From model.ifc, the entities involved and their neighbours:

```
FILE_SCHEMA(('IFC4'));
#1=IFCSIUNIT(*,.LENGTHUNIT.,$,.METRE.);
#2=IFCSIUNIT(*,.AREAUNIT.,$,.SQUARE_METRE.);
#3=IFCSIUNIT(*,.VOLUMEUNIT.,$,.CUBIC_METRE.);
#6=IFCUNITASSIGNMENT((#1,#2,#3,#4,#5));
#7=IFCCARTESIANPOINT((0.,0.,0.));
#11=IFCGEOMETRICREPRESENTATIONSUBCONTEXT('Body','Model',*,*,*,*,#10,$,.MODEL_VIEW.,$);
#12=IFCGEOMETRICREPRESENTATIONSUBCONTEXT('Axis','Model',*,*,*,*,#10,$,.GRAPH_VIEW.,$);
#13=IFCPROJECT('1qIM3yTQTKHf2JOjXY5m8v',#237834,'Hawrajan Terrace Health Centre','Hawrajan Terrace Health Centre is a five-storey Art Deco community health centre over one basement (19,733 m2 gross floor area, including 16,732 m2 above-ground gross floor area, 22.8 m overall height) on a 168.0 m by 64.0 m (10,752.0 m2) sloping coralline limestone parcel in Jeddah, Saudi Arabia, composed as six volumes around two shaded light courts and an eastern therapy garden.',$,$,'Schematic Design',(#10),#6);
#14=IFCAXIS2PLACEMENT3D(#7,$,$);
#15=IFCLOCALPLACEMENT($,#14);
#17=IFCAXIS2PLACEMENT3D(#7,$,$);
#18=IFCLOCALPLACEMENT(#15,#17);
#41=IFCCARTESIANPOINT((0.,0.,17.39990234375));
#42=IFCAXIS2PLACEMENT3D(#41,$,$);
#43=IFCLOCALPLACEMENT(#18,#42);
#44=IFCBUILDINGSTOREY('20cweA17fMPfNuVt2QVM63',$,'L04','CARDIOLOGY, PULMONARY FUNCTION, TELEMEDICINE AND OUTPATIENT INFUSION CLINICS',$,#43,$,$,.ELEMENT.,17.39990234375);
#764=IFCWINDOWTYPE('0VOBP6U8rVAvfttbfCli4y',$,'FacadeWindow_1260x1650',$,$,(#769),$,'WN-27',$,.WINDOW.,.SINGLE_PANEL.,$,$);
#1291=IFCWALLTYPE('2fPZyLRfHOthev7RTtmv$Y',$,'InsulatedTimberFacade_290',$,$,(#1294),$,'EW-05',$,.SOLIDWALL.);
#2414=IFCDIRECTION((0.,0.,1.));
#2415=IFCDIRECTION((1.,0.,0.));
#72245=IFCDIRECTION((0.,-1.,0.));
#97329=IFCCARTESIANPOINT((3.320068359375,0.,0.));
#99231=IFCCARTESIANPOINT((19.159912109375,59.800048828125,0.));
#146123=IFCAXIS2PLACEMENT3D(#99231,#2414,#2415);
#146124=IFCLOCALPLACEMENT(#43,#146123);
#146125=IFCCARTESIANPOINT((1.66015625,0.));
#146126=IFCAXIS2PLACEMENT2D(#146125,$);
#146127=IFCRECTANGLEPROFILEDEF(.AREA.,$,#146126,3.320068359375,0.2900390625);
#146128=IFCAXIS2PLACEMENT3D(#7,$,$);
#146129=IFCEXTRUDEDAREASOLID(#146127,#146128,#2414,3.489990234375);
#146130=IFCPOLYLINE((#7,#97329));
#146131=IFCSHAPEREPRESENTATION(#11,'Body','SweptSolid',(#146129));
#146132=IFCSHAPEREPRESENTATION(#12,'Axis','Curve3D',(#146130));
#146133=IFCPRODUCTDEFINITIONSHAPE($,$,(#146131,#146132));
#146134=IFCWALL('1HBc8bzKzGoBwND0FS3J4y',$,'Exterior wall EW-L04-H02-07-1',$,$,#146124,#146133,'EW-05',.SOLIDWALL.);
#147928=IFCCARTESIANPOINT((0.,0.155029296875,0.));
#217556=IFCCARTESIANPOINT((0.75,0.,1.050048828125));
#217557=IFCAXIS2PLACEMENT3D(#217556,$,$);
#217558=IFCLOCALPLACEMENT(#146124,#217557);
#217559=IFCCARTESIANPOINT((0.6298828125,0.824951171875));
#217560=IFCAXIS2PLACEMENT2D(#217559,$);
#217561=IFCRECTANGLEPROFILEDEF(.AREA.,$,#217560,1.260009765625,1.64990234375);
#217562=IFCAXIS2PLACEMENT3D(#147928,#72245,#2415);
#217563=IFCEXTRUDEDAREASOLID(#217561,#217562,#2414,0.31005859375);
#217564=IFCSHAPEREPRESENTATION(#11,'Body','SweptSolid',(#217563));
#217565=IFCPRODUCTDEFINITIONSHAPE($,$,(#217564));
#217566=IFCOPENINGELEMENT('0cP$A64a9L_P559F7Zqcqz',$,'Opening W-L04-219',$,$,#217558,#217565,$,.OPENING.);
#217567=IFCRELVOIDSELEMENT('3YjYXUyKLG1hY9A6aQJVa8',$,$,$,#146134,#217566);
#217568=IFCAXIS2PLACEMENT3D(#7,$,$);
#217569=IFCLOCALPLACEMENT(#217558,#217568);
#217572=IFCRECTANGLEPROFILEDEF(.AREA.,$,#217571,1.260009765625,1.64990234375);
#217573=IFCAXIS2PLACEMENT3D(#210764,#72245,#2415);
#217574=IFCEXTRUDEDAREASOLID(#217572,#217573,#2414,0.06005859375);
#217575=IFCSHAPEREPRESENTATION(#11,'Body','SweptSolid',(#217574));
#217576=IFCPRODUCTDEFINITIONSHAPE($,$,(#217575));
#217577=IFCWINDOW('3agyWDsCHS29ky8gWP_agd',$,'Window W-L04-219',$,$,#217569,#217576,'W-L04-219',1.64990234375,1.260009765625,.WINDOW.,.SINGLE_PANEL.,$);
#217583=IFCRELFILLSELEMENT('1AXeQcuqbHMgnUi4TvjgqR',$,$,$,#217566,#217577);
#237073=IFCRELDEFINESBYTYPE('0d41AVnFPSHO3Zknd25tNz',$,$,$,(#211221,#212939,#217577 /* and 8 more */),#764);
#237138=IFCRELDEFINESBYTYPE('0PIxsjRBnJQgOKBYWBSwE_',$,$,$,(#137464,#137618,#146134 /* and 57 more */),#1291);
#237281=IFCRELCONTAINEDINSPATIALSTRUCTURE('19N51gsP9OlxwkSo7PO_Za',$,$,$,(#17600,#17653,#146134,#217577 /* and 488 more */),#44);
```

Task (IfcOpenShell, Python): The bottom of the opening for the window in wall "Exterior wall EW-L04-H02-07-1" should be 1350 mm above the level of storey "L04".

```python
import numpy as np
import ifcopenshell
import ifcopenshell.api.geometry
import ifcopenshell.geom
import ifcopenshell.util.element
import ifcopenshell.util.placement
import ifcopenshell.util.shape
import ifcopenshell.util.unit

model = ifcopenshell.open("model.ifc")
unit_scale = ifcopenshell.util.unit.calculate_unit_scale(model)

window = model.by_guid("3agyWDsCHS29ky8gWP_agd")
opening = window.FillsVoids[0].RelatingOpeningElement
storey = ifcopenshell.util.element.get_container(window, ifc_class="IfcBuildingStorey")
level = ifcopenshell.util.placement.get_local_placement(storey.ObjectPlacement)[2, 3]

# The opening's origin need not be at the sill, so measure its lowest point.
shape = ifcopenshell.geom.create_shape(ifcopenshell.geom.settings(), opening)
bottom = ifcopenshell.util.shape.get_shape_bottom_elevation(shape, shape.geometry) / unit_scale
dz = level + 1.35 / unit_scale - bottom

shift = np.array([0.0, 0.0, dz])
# The window is placed relative to its opening, so it follows when the opening moves.
matrix = ifcopenshell.util.placement.get_local_placement(opening.ObjectPlacement)
matrix[:3, 3] += shift
ifcopenshell.api.geometry.edit_object_placement(
    model, product=opening, matrix=matrix, is_si=False, should_transform_children=True
)

print(f"moved by {dz * unit_scale:+.3f} m")

model.write("model_rev.ifc")
```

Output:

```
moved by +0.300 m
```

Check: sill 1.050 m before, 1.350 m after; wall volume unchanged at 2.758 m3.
